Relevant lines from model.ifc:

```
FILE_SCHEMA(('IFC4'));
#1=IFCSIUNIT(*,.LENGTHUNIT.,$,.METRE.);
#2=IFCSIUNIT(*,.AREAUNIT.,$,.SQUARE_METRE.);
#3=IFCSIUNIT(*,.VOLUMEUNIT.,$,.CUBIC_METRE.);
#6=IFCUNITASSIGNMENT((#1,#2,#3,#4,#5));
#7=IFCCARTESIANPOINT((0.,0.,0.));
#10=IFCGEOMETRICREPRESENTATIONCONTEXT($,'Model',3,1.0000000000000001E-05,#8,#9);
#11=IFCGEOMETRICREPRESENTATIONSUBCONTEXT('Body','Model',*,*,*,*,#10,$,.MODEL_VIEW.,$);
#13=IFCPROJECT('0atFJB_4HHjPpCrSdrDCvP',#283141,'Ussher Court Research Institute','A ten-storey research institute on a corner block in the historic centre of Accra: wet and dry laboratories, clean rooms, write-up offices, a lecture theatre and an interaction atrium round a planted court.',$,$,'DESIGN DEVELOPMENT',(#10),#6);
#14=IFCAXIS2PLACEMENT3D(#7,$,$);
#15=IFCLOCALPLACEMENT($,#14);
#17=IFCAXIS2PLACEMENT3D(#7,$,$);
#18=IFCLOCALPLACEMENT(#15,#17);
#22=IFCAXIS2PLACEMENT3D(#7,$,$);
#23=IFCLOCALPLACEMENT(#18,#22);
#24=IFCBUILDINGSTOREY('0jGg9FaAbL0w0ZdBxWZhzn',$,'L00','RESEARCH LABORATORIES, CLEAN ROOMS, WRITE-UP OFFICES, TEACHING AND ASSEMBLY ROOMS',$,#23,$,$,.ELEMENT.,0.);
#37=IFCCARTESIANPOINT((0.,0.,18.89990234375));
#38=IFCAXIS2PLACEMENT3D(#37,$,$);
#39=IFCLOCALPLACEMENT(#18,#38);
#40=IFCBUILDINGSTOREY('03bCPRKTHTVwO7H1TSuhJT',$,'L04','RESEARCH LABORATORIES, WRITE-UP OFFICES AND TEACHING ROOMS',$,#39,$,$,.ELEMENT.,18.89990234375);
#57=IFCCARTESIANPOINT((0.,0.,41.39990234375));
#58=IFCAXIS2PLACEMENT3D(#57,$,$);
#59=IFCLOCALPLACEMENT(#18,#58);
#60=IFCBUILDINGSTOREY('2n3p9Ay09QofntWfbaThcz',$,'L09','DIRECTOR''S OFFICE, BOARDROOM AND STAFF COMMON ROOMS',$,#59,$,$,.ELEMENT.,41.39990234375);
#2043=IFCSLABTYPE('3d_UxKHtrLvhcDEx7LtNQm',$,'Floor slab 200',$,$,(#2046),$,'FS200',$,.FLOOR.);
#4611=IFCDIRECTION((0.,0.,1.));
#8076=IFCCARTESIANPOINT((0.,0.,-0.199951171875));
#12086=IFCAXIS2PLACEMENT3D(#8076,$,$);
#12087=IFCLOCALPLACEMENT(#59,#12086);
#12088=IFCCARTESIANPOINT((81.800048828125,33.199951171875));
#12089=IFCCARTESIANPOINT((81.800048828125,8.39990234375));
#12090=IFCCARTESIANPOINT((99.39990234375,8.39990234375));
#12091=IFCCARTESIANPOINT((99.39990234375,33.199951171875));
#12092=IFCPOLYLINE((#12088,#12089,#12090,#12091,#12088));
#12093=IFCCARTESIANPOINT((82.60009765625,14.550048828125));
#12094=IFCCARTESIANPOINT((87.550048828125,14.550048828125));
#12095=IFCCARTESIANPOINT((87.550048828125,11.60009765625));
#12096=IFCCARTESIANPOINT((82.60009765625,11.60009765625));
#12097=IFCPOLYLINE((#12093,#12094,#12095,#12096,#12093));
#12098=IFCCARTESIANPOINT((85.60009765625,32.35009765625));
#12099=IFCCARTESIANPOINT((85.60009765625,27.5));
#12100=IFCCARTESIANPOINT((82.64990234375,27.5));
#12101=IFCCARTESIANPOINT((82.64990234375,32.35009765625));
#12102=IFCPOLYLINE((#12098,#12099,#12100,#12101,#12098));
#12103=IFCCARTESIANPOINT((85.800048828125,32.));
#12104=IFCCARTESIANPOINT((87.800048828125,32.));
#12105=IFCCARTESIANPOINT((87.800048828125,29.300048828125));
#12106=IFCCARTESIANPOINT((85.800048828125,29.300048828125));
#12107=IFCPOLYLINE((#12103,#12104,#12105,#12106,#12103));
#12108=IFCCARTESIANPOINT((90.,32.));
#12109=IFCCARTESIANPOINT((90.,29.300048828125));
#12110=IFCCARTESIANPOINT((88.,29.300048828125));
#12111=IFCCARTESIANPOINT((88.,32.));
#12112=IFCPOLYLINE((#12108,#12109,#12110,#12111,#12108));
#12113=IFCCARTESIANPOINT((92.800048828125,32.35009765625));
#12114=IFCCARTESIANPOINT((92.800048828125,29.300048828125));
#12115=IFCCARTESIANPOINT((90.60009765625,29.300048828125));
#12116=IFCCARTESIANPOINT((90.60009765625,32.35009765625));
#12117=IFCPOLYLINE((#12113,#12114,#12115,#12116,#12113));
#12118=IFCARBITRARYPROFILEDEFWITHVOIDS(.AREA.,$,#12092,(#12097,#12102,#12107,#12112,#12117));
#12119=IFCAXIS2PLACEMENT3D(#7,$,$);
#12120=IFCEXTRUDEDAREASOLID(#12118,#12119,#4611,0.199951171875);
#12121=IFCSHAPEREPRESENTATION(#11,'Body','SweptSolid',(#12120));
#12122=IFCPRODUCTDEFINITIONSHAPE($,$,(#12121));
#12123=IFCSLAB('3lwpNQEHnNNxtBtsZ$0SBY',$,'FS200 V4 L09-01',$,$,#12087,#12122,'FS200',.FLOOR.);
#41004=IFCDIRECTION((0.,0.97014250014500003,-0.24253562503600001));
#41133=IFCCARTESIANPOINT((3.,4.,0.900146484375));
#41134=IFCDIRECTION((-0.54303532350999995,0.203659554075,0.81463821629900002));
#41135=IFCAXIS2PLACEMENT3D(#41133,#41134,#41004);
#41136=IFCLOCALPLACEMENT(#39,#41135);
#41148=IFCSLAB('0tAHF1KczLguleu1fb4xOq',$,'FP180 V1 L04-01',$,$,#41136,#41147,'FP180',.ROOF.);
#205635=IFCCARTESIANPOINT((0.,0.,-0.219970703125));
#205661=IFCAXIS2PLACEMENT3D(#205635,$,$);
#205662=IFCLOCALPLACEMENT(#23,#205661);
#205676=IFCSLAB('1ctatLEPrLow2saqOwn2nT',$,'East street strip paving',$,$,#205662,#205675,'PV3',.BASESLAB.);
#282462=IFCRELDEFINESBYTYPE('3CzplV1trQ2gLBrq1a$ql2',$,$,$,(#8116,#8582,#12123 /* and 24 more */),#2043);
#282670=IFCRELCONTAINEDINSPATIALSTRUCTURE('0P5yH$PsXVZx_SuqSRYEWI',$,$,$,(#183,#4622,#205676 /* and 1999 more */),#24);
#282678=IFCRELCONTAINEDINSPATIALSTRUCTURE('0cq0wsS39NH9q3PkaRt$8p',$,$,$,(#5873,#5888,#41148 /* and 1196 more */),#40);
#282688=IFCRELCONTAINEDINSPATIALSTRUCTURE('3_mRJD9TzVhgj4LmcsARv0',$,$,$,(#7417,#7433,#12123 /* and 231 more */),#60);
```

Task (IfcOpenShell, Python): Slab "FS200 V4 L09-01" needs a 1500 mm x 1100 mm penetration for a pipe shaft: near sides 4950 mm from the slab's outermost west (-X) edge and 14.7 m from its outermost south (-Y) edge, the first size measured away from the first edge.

```python
import numpy as np
import ifcopenshell
import ifcopenshell.api.feature
import ifcopenshell.api.geometry
import ifcopenshell.api.root
import ifcopenshell.geom
import ifcopenshell.util.placement
import ifcopenshell.util.representation
import ifcopenshell.util.shape
import ifcopenshell.util.unit

model = ifcopenshell.open("model.ifc")
unit_scale = ifcopenshell.util.unit.calculate_unit_scale(model)
settings = ifcopenshell.geom.settings()


def volume(element):
    """Net volume in cubic metres, openings subtracted."""
    shape = ifcopenshell.geom.create_shape(settings, element)
    return ifcopenshell.util.shape.get_volume(shape.geometry)


slab = model.by_id(12123)
before = volume(slab)

# Extent in the slab's own axes, in metres. The edges named are its -X and -Y sides.
slab_shape = ifcopenshell.geom.create_shape(settings, slab)
vertices = ifcopenshell.util.shape.get_vertices(slab_shape.geometry)
x_min, y_min, bottom = vertices.min(axis=0)
top = vertices[:, 2].max()

opening = ifcopenshell.api.root.create_entity(model, ifc_class="IfcOpeningElement", name="Pipe shaft opening", predefined_type="OPENING")
context = ifcopenshell.util.representation.get_context(model, "Model", "Body", "MODEL_VIEW")
width, depth = 1.5, 1.1
outline = [(0.0, 0.0), (width, 0.0), (width, depth), (0.0, depth), (0.0, 0.0)]
# Overshoot both faces by 50 mm so the cut is clean.
shape = ifcopenshell.api.geometry.add_slab_representation(
    model, context=context, depth=top - bottom + 0.1, polyline=outline
)
ifcopenshell.api.geometry.assign_representation(model, product=opening, representation=shape)

matrix = ifcopenshell.util.placement.get_local_placement(slab.ObjectPlacement)
matrix[:, 3] = matrix @ np.append(np.array([x_min + 4.95, y_min + 14.7, bottom - 0.05]) / unit_scale, 1.0)
ifcopenshell.api.geometry.edit_object_placement(model, product=opening, matrix=matrix, is_si=False)
ifcopenshell.api.feature.add_feature(model, feature=opening, element=slab)

after = volume(slab)

print(f"slab volume {before:.3f} -> {after:.3f} m3")

model.write("model_rev.ifc")
```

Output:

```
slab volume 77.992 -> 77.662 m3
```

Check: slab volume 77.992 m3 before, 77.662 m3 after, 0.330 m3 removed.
